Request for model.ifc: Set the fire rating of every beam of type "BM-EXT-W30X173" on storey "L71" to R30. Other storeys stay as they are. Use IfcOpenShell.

First a look at what the model holds.

```python
import ifcopenshell
import ifcopenshell.util.element

model = ifcopenshell.open("model.ifc")
print(model.schema)
storey = next(s for s in model.by_type("IfcBuildingStorey") if s.Name == "L71")
beams = [e for e in ifcopenshell.util.element.get_decomposition(storey) if e.is_a("IfcBeam")]
seen = {}
for e in beams:
    element_type = ifcopenshell.util.element.get_type(e)
    key = (element_type.Name if element_type != e and element_type else None, ifcopenshell.util.element.get_pset(e, "Pset_BeamCommon", "FireRating"))
    seen[key] = seen.get(key, 0) + 1
for (name, value), count in sorted(seen.items(), key=str):
    print(count, "x", name, "|", value)
```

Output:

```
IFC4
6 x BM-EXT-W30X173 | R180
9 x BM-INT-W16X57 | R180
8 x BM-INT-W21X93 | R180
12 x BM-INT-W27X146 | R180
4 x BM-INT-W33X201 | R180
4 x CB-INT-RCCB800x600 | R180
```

```python
import ifcopenshell
import ifcopenshell.api.pset
import ifcopenshell.util.element

model = ifcopenshell.open("model.ifc")

storey = next(s for s in model.by_type("IfcBuildingStorey") if s.Name == "L71")
beams = [e for e in ifcopenshell.util.element.get_decomposition(storey) if e.is_a("IfcBeam")]

count = 0
for e in beams:
    element_type = ifcopenshell.util.element.get_type(e)
    if element_type in (None, e) or element_type.Name != "BM-EXT-W30X173":
        continue
    found = ifcopenshell.util.element.get_pset(e, "Pset_BeamCommon", should_inherit=False)
    if found:
        pset = model.by_id(found["id"])
        if len(ifcopenshell.util.element.get_elements_by_pset(pset)) > 1:
            pset = ifcopenshell.api.pset.unshare_pset(model, products=[e], pset=pset)[0]
    else:
        pset = ifcopenshell.api.pset.add_pset(model, product=e, name="Pset_BeamCommon")
    ifcopenshell.api.pset.edit_pset(model, pset=pset, properties={"FireRating": "R30"})
    count += 1

print(count, "beams updated")

model.write("model_rev.ifc")
```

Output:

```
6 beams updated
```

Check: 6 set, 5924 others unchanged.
